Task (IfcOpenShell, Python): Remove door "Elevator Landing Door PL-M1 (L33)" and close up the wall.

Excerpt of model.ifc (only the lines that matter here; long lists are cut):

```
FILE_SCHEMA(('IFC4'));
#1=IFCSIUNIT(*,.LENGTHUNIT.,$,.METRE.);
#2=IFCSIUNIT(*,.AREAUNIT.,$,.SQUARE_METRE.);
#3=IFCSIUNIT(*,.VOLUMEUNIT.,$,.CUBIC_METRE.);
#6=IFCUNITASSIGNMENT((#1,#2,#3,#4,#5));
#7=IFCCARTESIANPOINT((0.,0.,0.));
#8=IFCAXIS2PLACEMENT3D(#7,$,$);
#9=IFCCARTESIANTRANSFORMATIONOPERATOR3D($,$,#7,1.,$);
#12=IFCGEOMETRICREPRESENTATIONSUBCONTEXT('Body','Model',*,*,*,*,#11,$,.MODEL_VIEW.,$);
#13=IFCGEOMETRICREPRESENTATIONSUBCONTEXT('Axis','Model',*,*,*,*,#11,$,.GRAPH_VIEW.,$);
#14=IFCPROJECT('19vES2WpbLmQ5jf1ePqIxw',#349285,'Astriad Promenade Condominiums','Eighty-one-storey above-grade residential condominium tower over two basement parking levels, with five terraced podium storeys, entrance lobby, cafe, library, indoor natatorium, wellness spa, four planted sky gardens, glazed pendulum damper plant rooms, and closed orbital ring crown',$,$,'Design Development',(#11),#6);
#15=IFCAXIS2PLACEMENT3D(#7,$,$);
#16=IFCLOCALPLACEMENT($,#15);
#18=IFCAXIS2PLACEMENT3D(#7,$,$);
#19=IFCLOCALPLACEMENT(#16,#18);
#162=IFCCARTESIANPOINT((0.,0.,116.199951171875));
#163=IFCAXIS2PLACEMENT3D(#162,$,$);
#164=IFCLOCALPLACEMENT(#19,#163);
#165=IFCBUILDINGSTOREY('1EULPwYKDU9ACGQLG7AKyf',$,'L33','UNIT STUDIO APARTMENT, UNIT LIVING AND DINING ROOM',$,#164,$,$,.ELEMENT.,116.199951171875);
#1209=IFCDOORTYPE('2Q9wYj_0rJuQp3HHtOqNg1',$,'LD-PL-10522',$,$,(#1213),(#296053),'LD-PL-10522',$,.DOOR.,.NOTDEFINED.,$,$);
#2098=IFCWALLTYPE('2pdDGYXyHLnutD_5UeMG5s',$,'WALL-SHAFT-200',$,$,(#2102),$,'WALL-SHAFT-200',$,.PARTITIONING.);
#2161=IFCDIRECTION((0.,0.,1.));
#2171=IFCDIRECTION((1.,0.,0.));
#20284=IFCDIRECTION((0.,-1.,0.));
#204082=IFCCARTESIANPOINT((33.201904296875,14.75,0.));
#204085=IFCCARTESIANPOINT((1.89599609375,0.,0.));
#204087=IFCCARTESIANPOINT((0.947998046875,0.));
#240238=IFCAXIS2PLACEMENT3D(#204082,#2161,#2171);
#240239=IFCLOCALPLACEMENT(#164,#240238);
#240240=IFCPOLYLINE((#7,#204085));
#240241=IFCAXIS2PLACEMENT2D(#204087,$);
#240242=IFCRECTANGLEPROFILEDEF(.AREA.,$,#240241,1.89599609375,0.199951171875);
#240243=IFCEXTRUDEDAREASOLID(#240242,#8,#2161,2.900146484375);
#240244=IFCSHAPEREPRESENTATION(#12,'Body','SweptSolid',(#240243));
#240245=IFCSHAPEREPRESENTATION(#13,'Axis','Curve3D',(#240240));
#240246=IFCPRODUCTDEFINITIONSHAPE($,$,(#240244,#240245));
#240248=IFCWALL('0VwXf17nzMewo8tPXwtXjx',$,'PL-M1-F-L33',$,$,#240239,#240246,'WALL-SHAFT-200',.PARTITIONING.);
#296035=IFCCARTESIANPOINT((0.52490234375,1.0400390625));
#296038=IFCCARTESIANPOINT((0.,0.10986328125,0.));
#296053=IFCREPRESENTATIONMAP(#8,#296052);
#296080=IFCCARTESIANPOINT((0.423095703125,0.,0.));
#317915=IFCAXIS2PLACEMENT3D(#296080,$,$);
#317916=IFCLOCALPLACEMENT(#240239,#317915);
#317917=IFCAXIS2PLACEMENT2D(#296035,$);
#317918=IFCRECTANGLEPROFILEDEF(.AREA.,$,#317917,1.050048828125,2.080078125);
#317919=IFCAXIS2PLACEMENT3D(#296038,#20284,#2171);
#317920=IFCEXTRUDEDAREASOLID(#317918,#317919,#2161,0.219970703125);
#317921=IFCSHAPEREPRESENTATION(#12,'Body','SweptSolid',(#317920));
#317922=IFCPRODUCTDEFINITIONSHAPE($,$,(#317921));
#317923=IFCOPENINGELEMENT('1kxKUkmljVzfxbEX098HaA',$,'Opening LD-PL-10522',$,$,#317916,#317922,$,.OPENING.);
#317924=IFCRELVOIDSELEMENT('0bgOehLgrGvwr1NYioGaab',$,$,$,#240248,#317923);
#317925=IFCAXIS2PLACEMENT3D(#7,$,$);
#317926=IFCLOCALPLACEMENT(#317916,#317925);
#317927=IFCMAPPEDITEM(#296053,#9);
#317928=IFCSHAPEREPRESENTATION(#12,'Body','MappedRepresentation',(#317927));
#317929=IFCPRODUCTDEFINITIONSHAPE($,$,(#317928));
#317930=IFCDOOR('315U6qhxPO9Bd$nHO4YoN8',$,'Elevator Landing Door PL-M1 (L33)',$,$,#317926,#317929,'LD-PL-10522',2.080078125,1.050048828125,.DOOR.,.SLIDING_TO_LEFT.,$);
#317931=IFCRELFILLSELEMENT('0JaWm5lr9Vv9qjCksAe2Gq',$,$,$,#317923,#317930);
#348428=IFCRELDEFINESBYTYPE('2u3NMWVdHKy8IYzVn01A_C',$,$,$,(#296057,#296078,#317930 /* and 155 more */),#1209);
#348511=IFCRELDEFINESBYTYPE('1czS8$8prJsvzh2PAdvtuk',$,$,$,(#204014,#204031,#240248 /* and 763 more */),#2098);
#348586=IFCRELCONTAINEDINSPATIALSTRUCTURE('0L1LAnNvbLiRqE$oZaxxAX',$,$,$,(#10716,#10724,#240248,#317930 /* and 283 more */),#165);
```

```python
import ifcopenshell
import ifcopenshell.api.feature
import ifcopenshell.api.root
import ifcopenshell.geom
import ifcopenshell.util.shape

model = ifcopenshell.open("model.ifc")
settings = ifcopenshell.geom.settings()


def volume(element):
    """Net volume in cubic metres, openings subtracted."""
    shape = ifcopenshell.geom.create_shape(settings, element)
    return ifcopenshell.util.shape.get_volume(shape.geometry)


door = model.by_guid("315U6qhxPO9Bd$nHO4YoN8")
opening = door.FillsVoids[0].RelatingOpeningElement
wall = opening.VoidsElements[0].RelatingBuildingElement
before = volume(wall)

ifcopenshell.api.root.remove_product(model, product=door)
ifcopenshell.api.feature.remove_feature(model, feature=opening)

after = volume(wall)

print(f"wall volume {before:.3f} -> {after:.3f} m3")

model.write("model_rev.ifc")
```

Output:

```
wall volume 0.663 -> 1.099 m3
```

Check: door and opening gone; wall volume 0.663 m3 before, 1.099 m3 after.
